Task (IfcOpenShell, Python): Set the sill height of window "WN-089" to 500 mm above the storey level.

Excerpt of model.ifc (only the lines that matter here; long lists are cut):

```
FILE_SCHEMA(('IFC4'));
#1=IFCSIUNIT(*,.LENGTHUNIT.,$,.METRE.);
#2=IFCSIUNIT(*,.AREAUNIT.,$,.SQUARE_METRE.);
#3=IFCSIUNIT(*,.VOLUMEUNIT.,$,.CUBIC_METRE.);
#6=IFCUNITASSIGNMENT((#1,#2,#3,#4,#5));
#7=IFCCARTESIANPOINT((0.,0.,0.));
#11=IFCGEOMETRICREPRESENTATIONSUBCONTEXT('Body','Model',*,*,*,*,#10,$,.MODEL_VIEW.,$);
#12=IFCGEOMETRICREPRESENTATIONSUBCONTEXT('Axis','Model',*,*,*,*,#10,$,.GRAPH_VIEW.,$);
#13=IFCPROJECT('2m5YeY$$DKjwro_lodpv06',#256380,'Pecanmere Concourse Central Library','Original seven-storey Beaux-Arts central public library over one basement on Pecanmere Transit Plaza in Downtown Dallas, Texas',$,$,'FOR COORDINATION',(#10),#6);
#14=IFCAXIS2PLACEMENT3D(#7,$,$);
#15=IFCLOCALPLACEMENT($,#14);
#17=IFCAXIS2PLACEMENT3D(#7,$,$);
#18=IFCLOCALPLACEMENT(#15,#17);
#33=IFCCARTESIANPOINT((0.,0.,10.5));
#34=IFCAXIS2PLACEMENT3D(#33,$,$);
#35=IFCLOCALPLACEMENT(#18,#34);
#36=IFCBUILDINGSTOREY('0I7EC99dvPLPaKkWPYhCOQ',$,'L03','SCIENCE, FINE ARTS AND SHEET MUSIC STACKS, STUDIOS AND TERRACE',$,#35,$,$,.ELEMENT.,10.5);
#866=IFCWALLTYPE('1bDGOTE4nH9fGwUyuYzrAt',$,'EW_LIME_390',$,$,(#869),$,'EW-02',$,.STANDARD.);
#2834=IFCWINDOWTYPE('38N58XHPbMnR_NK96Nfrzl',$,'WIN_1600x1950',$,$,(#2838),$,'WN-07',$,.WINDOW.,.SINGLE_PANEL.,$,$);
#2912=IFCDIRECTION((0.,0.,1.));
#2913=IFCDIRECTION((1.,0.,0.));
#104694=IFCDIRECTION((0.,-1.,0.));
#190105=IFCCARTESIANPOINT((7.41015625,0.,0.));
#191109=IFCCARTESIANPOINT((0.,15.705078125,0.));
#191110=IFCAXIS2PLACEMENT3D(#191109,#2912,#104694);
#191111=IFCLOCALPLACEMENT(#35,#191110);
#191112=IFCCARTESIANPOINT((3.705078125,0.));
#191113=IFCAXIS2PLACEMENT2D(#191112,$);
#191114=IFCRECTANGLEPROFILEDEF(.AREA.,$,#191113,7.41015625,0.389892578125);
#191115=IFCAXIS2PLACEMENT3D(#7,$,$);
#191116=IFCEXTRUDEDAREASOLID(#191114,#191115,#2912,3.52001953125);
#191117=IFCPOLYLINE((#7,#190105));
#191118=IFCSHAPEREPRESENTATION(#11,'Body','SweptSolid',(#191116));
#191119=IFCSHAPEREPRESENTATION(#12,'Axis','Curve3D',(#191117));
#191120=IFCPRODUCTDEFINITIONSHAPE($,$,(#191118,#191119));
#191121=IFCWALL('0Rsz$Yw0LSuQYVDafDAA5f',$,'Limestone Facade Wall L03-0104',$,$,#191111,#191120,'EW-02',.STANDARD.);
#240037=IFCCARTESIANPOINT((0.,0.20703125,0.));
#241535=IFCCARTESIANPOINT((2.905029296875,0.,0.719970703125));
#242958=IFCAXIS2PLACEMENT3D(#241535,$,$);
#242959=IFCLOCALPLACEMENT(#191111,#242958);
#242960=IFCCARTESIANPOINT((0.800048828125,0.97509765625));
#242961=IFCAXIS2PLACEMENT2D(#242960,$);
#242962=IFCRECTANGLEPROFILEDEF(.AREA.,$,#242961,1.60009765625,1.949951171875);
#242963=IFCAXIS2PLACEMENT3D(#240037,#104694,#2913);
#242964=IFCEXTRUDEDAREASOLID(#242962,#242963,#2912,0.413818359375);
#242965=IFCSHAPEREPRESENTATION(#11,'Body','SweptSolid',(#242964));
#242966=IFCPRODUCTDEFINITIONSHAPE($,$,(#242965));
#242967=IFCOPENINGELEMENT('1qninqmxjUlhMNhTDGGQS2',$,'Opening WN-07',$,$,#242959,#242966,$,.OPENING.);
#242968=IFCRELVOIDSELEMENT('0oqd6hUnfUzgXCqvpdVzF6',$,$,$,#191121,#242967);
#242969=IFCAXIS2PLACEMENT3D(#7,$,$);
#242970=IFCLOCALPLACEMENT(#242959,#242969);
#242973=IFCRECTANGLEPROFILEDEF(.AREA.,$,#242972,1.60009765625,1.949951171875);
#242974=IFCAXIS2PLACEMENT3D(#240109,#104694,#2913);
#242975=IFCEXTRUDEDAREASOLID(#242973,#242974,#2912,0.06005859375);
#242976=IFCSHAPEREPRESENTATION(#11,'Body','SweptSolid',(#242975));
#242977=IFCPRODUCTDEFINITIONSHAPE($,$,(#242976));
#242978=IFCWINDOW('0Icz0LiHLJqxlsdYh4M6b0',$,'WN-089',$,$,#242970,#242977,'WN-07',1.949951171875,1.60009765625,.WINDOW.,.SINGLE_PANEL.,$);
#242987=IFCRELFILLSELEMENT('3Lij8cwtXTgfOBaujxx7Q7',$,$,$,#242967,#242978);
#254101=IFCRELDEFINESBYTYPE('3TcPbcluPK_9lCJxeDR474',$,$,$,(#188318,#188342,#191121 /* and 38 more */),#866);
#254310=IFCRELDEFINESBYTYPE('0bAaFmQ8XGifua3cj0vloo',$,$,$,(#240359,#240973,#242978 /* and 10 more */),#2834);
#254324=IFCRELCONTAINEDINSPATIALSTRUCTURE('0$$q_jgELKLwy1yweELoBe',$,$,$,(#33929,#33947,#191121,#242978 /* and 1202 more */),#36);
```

```python
import numpy as np
import ifcopenshell
import ifcopenshell.api.geometry
import ifcopenshell.geom
import ifcopenshell.util.element
import ifcopenshell.util.placement
import ifcopenshell.util.shape
import ifcopenshell.util.unit

model = ifcopenshell.open("model.ifc")
unit_scale = ifcopenshell.util.unit.calculate_unit_scale(model)

window = model.by_guid("0Icz0LiHLJqxlsdYh4M6b0")
opening = window.FillsVoids[0].RelatingOpeningElement
storey = ifcopenshell.util.element.get_container(window, ifc_class="IfcBuildingStorey")
level = ifcopenshell.util.placement.get_local_placement(storey.ObjectPlacement)[2, 3]

# The opening's origin need not be at the sill, so measure its lowest point.
shape = ifcopenshell.geom.create_shape(ifcopenshell.geom.settings(), opening)
bottom = ifcopenshell.util.shape.get_shape_bottom_elevation(shape, shape.geometry) / unit_scale
dz = level + 0.5 / unit_scale - bottom

shift = np.array([0.0, 0.0, dz])
# The window is placed relative to its opening, so it follows when the opening moves.
matrix = ifcopenshell.util.placement.get_local_placement(opening.ObjectPlacement)
matrix[:3, 3] += shift
ifcopenshell.api.geometry.edit_object_placement(
    model, product=opening, matrix=matrix, is_si=False, should_transform_children=True
)

print(f"moved by {dz * unit_scale:+.3f} m")

model.write("model_rev.ifc")
```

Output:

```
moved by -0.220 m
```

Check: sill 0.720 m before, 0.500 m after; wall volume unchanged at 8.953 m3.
